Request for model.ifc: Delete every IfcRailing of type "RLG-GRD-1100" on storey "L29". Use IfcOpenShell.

First a look at what the model holds.

```python
import ifcopenshell
import ifcopenshell.util.element

model = ifcopenshell.open("model.ifc")
print(model.schema)
storey = next(s for s in model.by_type("IfcBuildingStorey") if s.Name == "L29")
railings = [e for e in ifcopenshell.util.element.get_decomposition(storey) if e.is_a("IfcRailing")]
seen = {}
for e in railings:
    element_type = ifcopenshell.util.element.get_type(e)
    name = element_type.Name if element_type not in (None, e) else None
    seen[name] = seen.get(name, 0) + 1
for name, count in sorted(seen.items(), key=str):
    print(count, "x", name)
```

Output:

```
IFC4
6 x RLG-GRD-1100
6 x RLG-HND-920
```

```python
import ifcopenshell
import ifcopenshell.api.root
import ifcopenshell.util.element

model = ifcopenshell.open("model.ifc")

storey = next(s for s in model.by_type("IfcBuildingStorey") if s.Name == "L29")
railings = [e for e in ifcopenshell.util.element.get_decomposition(storey) if e.is_a("IfcRailing")]
targets = [e for e in railings if (t := ifcopenshell.util.element.get_type(e)) not in (None, e) and t.Name == "RLG-GRD-1100"]

for e in targets:
    ifcopenshell.api.root.remove_product(model, product=e)
print(len(targets), "removed")

model.write("model_updated.ifc")
```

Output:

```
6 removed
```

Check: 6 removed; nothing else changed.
